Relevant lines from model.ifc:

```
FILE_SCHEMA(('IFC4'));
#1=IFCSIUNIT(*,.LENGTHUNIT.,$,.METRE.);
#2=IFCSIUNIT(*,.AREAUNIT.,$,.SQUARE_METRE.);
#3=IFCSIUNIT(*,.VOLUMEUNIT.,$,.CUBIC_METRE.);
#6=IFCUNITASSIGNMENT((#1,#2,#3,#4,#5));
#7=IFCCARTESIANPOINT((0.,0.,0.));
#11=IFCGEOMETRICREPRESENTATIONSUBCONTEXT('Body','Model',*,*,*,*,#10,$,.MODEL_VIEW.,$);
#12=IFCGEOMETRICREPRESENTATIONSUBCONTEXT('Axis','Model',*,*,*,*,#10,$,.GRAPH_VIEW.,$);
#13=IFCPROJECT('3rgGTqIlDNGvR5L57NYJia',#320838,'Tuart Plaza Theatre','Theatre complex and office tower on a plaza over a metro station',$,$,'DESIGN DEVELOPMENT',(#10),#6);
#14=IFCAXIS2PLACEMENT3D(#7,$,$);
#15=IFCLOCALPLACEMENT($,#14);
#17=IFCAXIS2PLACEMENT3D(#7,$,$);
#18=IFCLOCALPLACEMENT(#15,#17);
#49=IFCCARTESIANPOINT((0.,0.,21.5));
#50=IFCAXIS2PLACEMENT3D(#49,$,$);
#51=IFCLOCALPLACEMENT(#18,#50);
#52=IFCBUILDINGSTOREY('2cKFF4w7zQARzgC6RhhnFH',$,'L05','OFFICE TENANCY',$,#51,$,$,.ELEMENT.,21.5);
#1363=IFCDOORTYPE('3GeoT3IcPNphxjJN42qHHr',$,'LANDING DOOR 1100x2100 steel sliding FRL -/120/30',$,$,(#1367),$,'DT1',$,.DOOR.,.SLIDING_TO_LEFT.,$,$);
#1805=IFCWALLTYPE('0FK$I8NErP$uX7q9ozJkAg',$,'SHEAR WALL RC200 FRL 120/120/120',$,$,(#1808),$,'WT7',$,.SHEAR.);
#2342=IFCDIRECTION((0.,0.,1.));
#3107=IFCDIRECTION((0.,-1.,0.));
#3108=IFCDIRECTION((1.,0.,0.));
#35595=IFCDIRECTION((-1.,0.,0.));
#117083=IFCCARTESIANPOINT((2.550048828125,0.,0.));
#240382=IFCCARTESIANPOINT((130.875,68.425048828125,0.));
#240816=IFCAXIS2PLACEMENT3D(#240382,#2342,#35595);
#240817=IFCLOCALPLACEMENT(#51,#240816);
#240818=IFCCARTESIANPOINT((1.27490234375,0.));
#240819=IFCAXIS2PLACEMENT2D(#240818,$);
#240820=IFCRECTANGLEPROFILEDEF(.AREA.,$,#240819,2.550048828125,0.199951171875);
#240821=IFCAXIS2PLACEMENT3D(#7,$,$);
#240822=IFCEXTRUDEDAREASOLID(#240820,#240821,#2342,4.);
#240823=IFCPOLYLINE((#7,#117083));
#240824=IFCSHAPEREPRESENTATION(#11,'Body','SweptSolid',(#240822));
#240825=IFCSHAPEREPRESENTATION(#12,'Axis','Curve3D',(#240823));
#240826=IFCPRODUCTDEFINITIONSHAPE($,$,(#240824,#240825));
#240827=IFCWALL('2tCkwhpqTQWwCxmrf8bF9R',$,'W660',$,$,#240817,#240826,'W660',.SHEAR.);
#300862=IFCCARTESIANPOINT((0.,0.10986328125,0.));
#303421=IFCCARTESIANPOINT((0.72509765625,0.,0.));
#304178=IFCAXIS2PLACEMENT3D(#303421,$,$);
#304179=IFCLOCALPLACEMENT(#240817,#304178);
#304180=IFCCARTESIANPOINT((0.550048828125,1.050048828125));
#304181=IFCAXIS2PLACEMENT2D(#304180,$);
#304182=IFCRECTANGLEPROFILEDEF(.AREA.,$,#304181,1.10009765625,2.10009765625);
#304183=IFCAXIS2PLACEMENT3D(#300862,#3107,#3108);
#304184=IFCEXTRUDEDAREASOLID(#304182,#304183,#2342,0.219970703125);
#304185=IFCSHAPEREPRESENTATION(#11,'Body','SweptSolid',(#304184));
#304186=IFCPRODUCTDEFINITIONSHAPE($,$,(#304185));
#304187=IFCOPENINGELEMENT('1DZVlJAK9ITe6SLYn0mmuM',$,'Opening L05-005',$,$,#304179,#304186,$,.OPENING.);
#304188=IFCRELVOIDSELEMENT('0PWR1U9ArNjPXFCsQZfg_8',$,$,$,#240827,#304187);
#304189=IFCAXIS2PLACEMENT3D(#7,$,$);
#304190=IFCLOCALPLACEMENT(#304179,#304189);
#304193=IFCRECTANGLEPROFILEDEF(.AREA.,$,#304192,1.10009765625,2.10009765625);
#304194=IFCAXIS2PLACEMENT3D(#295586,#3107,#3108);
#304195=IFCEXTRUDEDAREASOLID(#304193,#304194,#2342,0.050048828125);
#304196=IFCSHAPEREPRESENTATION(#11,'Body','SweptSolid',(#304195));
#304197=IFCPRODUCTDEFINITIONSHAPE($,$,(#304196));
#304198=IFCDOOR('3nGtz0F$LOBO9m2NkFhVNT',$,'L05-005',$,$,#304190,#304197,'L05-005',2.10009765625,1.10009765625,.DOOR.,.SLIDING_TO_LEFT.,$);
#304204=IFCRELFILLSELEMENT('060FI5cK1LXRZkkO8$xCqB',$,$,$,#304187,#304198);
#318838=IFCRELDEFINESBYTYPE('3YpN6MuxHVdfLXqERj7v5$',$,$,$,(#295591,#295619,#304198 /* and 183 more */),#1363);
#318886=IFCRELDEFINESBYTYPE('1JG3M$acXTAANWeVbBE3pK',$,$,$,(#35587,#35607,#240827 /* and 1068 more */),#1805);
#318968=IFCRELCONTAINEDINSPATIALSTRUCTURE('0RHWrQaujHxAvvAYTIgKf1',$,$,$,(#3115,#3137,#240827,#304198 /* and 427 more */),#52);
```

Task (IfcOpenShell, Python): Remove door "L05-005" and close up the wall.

```python
import ifcopenshell
import ifcopenshell.api.feature
import ifcopenshell.api.root
import ifcopenshell.geom
import ifcopenshell.util.shape

model = ifcopenshell.open("model.ifc")
settings = ifcopenshell.geom.settings()


def volume(element):
    """Net volume in cubic metres, openings subtracted."""
    shape = ifcopenshell.geom.create_shape(settings, element)
    return ifcopenshell.util.shape.get_volume(shape.geometry)


door = model.by_guid("3nGtz0F$LOBO9m2NkFhVNT")
opening = door.FillsVoids[0].RelatingOpeningElement
wall = opening.VoidsElements[0].RelatingBuildingElement
before = volume(wall)

ifcopenshell.api.root.remove_product(model, product=door)
ifcopenshell.api.feature.remove_feature(model, feature=opening)

after = volume(wall)

print(f"wall volume {before:.3f} -> {after:.3f} m3")

model.write("model_rev.ifc")
```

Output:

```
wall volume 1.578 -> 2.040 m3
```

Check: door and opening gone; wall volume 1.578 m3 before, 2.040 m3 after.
